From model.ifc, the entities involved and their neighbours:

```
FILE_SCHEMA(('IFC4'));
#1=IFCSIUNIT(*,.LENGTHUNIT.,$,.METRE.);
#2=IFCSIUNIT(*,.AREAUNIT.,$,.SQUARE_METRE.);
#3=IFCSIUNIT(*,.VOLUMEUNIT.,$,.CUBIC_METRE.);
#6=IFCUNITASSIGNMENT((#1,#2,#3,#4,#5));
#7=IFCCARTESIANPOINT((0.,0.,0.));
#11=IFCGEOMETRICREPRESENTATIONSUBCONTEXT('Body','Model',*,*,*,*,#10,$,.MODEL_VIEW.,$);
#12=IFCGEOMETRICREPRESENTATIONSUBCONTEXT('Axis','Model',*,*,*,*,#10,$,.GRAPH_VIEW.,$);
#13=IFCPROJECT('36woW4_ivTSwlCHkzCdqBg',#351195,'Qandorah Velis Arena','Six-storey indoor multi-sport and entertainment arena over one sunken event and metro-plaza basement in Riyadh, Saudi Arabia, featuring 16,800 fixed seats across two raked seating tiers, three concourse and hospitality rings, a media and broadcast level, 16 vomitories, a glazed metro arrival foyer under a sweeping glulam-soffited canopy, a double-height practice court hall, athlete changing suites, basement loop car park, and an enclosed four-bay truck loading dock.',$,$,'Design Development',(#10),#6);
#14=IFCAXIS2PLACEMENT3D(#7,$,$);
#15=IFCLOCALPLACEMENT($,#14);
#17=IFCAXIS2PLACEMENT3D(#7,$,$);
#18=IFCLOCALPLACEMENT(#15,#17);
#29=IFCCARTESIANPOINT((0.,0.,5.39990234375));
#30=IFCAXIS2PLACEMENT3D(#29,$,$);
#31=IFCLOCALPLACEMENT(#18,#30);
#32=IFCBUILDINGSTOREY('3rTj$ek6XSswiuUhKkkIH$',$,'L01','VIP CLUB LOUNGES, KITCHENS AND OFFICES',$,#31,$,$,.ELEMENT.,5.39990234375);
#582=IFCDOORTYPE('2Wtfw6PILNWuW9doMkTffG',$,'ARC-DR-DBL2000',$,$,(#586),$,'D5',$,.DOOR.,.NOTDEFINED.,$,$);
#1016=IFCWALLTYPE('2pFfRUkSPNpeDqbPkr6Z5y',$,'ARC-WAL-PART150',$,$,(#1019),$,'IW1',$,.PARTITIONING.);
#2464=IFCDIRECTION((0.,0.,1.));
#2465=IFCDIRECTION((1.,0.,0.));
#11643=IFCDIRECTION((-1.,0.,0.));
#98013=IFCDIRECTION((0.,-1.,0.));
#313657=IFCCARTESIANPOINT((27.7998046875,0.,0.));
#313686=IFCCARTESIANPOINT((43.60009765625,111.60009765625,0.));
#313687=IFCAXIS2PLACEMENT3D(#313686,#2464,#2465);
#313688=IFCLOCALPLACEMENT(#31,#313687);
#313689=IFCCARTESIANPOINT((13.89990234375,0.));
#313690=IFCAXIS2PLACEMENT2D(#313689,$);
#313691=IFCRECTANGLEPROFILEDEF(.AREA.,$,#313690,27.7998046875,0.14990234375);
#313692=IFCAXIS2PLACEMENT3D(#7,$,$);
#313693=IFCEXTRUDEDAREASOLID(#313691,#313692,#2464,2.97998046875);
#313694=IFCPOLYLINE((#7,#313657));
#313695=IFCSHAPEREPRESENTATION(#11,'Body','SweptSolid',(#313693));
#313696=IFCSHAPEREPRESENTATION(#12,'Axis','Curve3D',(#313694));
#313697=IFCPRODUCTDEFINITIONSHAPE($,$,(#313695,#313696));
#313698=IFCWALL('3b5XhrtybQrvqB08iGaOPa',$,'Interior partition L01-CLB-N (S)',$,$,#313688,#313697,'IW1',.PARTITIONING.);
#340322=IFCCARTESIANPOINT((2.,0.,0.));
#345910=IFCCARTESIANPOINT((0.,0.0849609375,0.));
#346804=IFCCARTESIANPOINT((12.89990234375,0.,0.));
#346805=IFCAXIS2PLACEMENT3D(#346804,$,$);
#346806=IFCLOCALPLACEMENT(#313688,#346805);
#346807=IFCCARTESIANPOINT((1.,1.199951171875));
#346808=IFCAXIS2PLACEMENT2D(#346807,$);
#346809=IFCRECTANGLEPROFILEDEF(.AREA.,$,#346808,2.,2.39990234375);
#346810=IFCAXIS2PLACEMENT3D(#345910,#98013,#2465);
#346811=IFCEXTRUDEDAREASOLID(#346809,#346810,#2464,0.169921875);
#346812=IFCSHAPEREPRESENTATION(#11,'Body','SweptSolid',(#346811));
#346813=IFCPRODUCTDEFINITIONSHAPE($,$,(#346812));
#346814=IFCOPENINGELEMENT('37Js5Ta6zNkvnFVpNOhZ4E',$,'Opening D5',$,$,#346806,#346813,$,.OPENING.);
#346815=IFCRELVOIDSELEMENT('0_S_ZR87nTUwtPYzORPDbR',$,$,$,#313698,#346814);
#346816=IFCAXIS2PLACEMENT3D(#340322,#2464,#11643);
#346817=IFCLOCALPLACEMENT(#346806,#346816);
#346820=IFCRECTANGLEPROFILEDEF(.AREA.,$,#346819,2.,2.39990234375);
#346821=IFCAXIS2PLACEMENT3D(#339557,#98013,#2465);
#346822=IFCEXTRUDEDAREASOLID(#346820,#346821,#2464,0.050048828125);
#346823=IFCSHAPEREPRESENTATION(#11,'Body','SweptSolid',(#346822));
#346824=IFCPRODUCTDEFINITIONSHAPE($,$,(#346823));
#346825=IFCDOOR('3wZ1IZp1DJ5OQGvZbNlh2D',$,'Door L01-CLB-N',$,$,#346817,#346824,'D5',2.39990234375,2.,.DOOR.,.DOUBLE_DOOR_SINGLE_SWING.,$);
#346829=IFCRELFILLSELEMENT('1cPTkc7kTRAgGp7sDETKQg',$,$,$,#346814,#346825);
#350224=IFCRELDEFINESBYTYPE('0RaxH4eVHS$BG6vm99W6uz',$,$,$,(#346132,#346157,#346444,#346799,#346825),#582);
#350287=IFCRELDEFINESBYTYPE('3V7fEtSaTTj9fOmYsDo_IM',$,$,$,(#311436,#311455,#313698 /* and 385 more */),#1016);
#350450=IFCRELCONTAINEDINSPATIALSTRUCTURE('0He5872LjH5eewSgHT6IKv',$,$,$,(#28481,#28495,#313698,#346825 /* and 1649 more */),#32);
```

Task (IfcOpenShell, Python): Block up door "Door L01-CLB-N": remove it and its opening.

```python
import ifcopenshell
import ifcopenshell.api.feature
import ifcopenshell.api.root
import ifcopenshell.geom
import ifcopenshell.util.shape

model = ifcopenshell.open("model.ifc")
settings = ifcopenshell.geom.settings()


def volume(element):
    """Net volume in cubic metres, openings subtracted."""
    shape = ifcopenshell.geom.create_shape(settings, element)
    return ifcopenshell.util.shape.get_volume(shape.geometry)


door = model.by_guid("3wZ1IZp1DJ5OQGvZbNlh2D")
opening = door.FillsVoids[0].RelatingOpeningElement
wall = opening.VoidsElements[0].RelatingBuildingElement
before = volume(wall)

ifcopenshell.api.root.remove_product(model, product=door)
ifcopenshell.api.feature.remove_feature(model, feature=opening)

after = volume(wall)

print(f"wall volume {before:.3f} -> {after:.3f} m3")

model.write("model_v2.ifc")
```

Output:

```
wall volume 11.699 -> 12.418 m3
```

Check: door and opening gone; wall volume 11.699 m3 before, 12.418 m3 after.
